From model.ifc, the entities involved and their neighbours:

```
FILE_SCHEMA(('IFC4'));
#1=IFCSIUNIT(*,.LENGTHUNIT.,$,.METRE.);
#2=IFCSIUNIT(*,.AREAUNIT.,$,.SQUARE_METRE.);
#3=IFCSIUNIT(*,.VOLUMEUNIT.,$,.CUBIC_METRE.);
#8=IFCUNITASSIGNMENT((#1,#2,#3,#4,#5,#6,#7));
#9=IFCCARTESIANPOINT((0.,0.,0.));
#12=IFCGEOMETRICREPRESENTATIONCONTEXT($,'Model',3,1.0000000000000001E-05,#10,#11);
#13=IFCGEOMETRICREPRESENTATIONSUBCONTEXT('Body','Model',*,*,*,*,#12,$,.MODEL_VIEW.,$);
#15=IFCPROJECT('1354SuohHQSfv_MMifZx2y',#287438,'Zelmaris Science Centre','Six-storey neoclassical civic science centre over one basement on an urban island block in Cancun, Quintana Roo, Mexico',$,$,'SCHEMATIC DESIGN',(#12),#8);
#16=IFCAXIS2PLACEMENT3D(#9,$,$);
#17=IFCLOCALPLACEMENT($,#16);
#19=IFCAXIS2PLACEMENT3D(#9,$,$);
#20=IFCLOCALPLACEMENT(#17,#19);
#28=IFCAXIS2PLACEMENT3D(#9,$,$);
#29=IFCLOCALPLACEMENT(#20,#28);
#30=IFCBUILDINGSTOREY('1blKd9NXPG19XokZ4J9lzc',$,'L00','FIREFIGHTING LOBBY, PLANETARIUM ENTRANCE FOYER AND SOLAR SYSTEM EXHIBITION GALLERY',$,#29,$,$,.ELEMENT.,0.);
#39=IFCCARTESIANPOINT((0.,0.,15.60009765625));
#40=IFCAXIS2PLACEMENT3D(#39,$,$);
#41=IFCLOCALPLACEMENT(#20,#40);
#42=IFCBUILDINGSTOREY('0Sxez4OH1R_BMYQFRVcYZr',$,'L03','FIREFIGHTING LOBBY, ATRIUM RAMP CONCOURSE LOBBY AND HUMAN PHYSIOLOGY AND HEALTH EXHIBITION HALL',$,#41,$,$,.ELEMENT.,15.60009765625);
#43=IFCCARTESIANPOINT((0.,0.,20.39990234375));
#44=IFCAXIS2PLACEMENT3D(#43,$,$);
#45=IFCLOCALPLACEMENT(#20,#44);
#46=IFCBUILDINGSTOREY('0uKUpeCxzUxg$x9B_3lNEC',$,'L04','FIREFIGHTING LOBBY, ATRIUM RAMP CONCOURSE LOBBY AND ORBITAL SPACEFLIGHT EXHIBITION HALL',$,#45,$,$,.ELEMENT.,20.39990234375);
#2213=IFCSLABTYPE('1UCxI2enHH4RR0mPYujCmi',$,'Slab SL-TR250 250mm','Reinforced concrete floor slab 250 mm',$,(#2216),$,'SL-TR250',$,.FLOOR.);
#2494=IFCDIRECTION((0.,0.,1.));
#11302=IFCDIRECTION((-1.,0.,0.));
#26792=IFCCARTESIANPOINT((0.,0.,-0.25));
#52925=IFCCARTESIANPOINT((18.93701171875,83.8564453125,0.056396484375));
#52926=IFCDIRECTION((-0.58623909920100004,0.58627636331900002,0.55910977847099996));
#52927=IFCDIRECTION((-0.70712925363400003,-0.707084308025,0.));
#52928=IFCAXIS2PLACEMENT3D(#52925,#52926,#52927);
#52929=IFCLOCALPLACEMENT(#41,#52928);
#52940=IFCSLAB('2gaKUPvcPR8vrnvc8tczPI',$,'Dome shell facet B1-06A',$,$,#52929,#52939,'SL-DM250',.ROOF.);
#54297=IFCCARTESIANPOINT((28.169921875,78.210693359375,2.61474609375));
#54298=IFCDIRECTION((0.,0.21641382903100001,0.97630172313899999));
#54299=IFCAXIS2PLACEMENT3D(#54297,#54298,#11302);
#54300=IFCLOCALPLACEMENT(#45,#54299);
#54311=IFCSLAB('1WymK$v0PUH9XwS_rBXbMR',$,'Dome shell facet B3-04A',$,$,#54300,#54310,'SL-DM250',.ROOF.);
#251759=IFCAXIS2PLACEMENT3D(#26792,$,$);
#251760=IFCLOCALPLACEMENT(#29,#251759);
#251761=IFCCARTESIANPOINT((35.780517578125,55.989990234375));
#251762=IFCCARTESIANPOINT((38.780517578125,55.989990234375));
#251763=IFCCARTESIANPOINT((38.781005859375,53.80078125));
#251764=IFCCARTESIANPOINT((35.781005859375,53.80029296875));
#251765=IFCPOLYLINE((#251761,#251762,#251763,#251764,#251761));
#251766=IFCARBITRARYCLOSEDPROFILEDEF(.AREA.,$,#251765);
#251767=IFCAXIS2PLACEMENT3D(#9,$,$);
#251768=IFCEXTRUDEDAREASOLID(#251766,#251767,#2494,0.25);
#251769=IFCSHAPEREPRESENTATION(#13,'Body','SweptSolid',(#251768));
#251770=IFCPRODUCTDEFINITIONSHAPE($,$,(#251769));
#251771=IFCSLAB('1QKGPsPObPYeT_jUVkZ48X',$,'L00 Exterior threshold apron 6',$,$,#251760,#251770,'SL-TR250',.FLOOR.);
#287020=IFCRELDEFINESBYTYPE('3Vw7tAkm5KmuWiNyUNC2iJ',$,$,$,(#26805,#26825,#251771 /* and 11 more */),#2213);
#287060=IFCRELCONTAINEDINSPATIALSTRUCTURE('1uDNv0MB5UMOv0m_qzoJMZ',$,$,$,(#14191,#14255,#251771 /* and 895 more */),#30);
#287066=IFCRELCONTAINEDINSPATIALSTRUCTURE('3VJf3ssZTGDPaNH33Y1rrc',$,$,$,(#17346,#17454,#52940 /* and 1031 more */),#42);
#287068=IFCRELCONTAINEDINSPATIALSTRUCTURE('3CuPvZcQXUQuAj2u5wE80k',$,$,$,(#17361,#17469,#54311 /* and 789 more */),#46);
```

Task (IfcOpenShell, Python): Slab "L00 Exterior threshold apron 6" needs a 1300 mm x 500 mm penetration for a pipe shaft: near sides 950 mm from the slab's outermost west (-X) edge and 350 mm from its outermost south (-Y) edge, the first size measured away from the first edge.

```python
import numpy as np
import ifcopenshell
import ifcopenshell.api.feature
import ifcopenshell.api.geometry
import ifcopenshell.api.root
import ifcopenshell.geom
import ifcopenshell.util.placement
import ifcopenshell.util.representation
import ifcopenshell.util.shape
import ifcopenshell.util.unit

model = ifcopenshell.open("model.ifc")
unit_scale = ifcopenshell.util.unit.calculate_unit_scale(model)
settings = ifcopenshell.geom.settings()


def volume(element):
    """Net volume in cubic metres, openings subtracted."""
    shape = ifcopenshell.geom.create_shape(settings, element)
    return ifcopenshell.util.shape.get_volume(shape.geometry)


slab = model.by_guid("1QKGPsPObPYeT_jUVkZ48X")
before = volume(slab)

# Extent in the slab's own axes, in metres. The edges named are its -X and -Y sides.
slab_shape = ifcopenshell.geom.create_shape(settings, slab)
vertices = ifcopenshell.util.shape.get_vertices(slab_shape.geometry)
x_min, y_min, bottom = vertices.min(axis=0)
top = vertices[:, 2].max()

opening = ifcopenshell.api.root.create_entity(model, ifc_class="IfcOpeningElement", name="Pipe shaft opening", predefined_type="OPENING")
context = ifcopenshell.util.representation.get_context(model, "Model", "Body", "MODEL_VIEW")
width, depth = 1.3, 0.5
outline = [(0.0, 0.0), (width, 0.0), (width, depth), (0.0, depth), (0.0, 0.0)]
# Overshoot both faces by 50 mm so the cut is clean.
shape = ifcopenshell.api.geometry.add_slab_representation(
    model, context=context, depth=top - bottom + 0.1, polyline=outline
)
ifcopenshell.api.geometry.assign_representation(model, product=opening, representation=shape)

matrix = ifcopenshell.util.placement.get_local_placement(slab.ObjectPlacement)
matrix[:, 3] = matrix @ np.append(np.array([x_min + 0.95, y_min + 0.35, bottom - 0.05]) / unit_scale, 1.0)
ifcopenshell.api.geometry.edit_object_placement(model, product=opening, matrix=matrix, is_si=False)
ifcopenshell.api.feature.add_feature(model, feature=opening, element=slab)

after = volume(slab)

print(f"slab volume {before:.3f} -> {after:.3f} m3")

model.write("model-out.ifc")
```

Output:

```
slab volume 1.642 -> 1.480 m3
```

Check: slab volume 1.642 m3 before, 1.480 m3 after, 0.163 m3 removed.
